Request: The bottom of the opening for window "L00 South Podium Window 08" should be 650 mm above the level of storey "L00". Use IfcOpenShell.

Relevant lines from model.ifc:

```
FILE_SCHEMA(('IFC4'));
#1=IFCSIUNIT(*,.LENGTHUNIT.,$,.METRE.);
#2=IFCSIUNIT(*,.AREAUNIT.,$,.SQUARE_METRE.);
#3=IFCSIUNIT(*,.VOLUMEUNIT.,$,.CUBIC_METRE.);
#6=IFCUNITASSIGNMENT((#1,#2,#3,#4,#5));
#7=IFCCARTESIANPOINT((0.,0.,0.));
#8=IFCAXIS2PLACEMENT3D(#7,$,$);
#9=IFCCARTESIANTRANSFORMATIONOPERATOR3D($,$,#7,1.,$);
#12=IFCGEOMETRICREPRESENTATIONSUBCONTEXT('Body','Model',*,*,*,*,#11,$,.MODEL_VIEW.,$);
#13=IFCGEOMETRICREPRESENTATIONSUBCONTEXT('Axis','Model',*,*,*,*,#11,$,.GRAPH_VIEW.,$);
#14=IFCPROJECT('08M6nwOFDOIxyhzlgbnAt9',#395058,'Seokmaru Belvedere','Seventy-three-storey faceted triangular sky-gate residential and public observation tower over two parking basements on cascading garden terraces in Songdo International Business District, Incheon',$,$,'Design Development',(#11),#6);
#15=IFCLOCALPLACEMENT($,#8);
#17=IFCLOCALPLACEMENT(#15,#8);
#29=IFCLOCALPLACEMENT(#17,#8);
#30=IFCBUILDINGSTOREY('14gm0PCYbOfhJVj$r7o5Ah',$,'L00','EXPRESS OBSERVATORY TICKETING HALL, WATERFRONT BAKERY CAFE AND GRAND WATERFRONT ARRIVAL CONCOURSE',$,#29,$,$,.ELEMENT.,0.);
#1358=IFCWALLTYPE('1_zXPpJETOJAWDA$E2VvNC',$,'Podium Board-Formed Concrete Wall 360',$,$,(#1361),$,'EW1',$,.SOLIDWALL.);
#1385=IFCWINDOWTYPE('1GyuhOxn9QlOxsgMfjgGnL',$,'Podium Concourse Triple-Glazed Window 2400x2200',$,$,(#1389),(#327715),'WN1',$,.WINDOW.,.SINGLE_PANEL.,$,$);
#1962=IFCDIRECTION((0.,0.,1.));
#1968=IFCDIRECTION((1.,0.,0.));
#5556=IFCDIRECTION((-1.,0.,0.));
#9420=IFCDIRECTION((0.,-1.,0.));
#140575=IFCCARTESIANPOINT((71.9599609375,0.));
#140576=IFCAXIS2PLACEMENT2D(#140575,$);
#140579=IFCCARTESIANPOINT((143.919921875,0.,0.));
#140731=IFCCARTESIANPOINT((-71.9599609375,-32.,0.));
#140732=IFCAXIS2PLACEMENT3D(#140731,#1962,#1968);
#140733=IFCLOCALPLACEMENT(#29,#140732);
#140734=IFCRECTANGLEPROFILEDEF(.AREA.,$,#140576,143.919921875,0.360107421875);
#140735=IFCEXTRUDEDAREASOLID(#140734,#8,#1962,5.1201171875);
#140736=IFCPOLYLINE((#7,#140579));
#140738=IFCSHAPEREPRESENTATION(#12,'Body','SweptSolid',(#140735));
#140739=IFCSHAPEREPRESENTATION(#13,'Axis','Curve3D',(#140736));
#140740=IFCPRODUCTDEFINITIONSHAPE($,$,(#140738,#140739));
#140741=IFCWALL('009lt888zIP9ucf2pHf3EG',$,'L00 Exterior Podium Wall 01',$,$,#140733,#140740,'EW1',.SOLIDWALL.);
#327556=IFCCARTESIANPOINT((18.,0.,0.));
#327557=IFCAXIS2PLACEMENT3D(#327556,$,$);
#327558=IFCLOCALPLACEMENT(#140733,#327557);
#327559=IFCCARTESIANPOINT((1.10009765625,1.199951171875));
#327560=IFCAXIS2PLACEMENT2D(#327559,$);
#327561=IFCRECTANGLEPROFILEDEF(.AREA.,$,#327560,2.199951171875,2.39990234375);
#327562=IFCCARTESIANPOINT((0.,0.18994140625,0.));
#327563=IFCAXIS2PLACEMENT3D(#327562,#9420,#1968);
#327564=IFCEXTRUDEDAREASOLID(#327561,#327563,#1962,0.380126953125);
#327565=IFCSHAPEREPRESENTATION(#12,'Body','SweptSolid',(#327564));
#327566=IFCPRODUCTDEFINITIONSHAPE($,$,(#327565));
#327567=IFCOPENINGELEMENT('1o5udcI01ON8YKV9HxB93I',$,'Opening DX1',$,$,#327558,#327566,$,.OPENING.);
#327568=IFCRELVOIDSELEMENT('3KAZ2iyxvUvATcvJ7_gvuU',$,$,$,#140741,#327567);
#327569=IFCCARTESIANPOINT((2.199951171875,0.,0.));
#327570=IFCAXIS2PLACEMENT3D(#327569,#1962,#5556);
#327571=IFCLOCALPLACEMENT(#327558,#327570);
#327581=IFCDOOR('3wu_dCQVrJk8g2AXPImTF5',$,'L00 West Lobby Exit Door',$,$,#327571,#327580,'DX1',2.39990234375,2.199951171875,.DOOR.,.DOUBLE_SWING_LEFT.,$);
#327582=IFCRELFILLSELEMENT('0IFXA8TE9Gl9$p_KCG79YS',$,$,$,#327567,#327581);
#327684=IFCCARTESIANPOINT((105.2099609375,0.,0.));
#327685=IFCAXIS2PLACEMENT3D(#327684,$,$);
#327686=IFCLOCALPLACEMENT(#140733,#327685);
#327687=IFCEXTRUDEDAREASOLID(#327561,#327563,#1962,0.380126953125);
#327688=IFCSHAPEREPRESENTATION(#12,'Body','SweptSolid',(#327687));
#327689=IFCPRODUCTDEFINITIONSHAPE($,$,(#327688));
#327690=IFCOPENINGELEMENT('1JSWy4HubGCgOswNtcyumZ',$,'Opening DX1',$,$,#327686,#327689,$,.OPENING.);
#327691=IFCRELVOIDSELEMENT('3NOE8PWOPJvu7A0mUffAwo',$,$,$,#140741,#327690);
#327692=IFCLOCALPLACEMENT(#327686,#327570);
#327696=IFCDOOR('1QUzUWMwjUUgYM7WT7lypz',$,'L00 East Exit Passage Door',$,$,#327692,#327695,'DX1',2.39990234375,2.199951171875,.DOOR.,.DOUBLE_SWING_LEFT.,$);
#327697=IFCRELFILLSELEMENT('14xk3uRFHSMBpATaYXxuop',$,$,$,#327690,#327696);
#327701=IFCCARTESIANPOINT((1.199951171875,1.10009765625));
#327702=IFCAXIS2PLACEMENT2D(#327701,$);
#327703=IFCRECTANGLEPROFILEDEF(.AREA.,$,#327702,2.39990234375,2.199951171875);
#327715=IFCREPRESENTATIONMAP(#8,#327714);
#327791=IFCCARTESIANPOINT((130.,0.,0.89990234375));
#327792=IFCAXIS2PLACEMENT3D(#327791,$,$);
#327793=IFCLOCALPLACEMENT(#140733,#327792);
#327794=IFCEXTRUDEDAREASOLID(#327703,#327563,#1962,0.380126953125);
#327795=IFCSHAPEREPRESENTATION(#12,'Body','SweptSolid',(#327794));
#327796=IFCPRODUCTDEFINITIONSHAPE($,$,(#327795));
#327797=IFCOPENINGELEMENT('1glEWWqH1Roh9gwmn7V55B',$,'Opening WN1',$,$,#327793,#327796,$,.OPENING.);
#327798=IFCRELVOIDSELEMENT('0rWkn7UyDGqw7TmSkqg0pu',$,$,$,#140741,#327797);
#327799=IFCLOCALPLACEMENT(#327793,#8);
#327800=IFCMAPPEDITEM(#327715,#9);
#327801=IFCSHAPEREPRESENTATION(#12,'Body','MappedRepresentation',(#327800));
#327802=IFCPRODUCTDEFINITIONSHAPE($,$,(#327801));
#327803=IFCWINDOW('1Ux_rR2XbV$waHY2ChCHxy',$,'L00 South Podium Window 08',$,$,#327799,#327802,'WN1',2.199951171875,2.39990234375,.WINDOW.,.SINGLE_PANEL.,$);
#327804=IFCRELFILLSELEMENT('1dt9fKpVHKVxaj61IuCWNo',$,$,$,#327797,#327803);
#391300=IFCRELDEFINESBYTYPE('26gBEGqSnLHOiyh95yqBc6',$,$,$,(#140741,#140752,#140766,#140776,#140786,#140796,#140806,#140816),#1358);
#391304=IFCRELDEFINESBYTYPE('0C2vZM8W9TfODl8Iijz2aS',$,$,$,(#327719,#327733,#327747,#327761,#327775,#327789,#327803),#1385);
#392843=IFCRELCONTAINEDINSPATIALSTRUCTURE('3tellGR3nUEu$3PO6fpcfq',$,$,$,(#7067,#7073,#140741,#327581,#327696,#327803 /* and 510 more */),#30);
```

```python
import numpy as np
import ifcopenshell
import ifcopenshell.api.geometry
import ifcopenshell.geom
import ifcopenshell.util.element
import ifcopenshell.util.placement
import ifcopenshell.util.shape
import ifcopenshell.util.unit

model = ifcopenshell.open("model.ifc")
unit_scale = ifcopenshell.util.unit.calculate_unit_scale(model)

window = model.by_guid("1Ux_rR2XbV$waHY2ChCHxy")
opening = window.FillsVoids[0].RelatingOpeningElement
storey = ifcopenshell.util.element.get_container(window, ifc_class="IfcBuildingStorey")
level = ifcopenshell.util.placement.get_local_placement(storey.ObjectPlacement)[2, 3]

# The opening's origin need not be at the sill, so measure its lowest point.
shape = ifcopenshell.geom.create_shape(ifcopenshell.geom.settings(), opening)
bottom = ifcopenshell.util.shape.get_shape_bottom_elevation(shape, shape.geometry) / unit_scale
dz = level + 0.65 - bottom

shift = np.array([0.0, 0.0, dz])
# The window is placed relative to its opening, so it follows when the opening moves.
matrix = ifcopenshell.util.placement.get_local_placement(opening.ObjectPlacement)
matrix[:3, 3] += shift
ifcopenshell.api.geometry.edit_object_placement(
    model, product=opening, matrix=matrix, is_si=False, should_transform_children=True
)

print(f"moved by {dz * unit_scale:+.3f} m")

model.write("model-out.ifc")
```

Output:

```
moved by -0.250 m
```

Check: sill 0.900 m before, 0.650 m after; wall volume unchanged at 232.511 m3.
